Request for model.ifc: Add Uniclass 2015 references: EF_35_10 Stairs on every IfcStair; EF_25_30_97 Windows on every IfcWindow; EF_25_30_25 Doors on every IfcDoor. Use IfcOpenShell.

First a look at what the model holds.

```python
import ifcopenshell

model = ifcopenshell.open("model.ifc")
print(model.schema)
print("classifications:", [c.Name for c in model.by_type("IfcClassification")])
for ifc_class in ("IfcDoor", "IfcRoof", "IfcStair", "IfcWall", "IfcWindow"):
    print(ifc_class, len(model.by_type(ifc_class)))
```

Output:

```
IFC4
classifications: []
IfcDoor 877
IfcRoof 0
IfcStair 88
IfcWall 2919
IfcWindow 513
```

```python
import ifcopenshell
import ifcopenshell.api.classification

model = ifcopenshell.open("model.ifc")

system = ifcopenshell.api.classification.add_classification(model, classification="Uniclass 2015")

codes = {
    "IfcStair": ("EF_35_10", "Stairs"),
    "IfcWindow": ("EF_25_30_97", "Windows"),
    "IfcDoor": ("EF_25_30_25", "Doors"),
}
for ifc_class, (code, name) in codes.items():
    products = model.by_type(ifc_class)
    ifcopenshell.api.classification.add_reference(
        model, products=products, classification=system, identification=code, name=name
    )
    print(code, len(products))

model.write("model_rev.ifc")
```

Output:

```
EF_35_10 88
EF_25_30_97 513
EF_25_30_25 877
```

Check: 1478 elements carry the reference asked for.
